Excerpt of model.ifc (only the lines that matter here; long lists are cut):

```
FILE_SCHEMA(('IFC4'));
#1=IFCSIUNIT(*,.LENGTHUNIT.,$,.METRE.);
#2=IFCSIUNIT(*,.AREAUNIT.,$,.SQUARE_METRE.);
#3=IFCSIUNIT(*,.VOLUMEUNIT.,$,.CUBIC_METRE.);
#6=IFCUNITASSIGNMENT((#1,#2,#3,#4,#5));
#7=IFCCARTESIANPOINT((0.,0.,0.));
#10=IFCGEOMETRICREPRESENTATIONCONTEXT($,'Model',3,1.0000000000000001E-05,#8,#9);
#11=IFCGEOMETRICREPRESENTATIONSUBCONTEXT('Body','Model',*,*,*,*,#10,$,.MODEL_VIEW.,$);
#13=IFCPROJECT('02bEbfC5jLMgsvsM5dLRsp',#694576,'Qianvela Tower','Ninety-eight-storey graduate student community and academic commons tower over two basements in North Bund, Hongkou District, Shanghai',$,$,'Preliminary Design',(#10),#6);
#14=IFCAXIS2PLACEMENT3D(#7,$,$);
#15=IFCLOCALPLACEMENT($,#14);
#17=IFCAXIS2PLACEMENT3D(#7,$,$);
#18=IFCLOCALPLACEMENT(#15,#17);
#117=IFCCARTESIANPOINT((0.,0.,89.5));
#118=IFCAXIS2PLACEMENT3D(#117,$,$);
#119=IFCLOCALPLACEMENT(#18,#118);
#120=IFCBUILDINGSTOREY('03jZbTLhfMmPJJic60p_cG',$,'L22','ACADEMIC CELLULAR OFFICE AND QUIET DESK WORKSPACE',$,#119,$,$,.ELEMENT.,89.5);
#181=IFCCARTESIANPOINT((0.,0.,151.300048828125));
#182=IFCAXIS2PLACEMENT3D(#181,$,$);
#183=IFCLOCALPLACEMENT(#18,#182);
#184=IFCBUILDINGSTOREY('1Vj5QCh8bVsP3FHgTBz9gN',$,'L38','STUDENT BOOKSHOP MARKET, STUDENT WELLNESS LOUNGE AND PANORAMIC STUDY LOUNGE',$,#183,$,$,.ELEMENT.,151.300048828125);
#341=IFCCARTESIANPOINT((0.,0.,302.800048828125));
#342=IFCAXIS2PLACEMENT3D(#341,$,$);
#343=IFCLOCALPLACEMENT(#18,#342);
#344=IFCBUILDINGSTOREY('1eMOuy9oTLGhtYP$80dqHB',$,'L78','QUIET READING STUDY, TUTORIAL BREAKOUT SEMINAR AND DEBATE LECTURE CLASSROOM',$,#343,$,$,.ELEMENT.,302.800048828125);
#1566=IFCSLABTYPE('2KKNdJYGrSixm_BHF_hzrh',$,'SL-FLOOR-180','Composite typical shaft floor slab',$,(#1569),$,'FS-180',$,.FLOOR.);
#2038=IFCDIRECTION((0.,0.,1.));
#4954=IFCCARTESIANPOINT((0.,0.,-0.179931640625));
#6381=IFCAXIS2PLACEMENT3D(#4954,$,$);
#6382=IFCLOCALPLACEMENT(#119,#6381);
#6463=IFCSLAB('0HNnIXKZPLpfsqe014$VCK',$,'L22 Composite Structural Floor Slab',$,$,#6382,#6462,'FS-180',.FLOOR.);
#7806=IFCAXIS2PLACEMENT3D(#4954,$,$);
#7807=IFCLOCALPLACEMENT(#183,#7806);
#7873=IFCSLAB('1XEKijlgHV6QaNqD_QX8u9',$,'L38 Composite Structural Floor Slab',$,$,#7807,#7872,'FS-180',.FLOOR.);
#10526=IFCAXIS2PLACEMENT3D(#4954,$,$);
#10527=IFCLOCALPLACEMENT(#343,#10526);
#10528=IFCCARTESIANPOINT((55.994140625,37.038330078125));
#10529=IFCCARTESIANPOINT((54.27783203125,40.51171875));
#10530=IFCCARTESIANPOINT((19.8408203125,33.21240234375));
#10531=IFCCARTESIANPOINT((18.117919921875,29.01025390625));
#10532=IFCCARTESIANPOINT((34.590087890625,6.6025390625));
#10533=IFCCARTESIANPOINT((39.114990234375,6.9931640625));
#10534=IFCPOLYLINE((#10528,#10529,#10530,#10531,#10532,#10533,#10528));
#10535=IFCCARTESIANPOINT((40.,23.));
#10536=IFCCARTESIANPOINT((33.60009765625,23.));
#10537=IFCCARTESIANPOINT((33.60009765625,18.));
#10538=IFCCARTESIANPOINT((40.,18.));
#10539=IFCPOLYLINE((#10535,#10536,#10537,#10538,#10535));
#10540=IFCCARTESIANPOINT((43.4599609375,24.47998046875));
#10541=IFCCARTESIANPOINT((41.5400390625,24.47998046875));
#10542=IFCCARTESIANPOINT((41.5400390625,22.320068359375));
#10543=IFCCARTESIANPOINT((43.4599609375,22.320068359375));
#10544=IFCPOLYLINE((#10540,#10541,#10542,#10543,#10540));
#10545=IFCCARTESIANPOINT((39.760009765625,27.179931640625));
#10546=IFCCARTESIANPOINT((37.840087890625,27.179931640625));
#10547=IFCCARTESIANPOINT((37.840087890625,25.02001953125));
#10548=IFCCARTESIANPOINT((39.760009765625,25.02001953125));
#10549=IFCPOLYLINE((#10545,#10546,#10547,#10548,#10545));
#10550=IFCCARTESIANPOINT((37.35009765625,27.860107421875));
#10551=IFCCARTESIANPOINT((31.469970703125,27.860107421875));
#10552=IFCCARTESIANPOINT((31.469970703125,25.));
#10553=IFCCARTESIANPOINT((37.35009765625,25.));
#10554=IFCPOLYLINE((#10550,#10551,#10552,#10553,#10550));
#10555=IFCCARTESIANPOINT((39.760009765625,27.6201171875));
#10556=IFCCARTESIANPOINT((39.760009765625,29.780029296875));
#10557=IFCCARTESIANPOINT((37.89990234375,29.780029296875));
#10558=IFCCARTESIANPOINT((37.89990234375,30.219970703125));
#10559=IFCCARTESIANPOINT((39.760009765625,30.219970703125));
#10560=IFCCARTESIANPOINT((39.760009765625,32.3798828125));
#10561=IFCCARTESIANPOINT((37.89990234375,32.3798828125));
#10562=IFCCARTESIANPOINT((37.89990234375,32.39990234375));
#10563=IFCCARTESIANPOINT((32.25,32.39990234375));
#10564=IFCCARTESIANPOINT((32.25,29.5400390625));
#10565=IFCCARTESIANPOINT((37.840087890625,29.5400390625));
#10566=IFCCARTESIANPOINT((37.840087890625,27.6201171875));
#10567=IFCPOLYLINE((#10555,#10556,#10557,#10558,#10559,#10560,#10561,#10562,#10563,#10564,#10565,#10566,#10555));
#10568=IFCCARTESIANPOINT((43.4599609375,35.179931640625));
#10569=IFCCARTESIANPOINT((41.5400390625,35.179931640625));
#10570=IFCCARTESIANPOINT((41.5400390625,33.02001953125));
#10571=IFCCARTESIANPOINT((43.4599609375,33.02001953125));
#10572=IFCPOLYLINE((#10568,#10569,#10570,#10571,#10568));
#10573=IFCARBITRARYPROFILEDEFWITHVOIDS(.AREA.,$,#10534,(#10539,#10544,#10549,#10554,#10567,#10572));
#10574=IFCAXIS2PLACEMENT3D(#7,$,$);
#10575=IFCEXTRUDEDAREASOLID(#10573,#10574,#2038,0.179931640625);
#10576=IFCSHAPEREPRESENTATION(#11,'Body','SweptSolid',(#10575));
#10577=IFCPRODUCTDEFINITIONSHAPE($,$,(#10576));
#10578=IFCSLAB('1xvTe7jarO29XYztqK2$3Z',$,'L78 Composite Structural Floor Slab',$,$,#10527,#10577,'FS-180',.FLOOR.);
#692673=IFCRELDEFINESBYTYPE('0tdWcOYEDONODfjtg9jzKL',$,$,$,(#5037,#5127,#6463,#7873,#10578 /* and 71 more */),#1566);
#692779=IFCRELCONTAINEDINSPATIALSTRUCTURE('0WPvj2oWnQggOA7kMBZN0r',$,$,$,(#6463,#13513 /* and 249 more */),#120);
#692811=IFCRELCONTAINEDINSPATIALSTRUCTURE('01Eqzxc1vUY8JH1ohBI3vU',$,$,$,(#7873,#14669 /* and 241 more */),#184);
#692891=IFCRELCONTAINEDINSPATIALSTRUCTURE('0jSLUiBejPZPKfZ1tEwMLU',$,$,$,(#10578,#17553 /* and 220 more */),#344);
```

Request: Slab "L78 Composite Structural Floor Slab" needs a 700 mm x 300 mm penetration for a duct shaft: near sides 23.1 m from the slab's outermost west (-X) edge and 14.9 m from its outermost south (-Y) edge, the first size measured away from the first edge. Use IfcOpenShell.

```python
import numpy as np
import ifcopenshell
import ifcopenshell.api.feature
import ifcopenshell.api.geometry
import ifcopenshell.api.root
import ifcopenshell.geom
import ifcopenshell.util.placement
import ifcopenshell.util.representation
import ifcopenshell.util.shape
import ifcopenshell.util.unit

model = ifcopenshell.open("model.ifc")
unit_scale = ifcopenshell.util.unit.calculate_unit_scale(model)
settings = ifcopenshell.geom.settings()


def volume(element):
    """Net volume in cubic metres, openings subtracted."""
    shape = ifcopenshell.geom.create_shape(settings, element)
    return ifcopenshell.util.shape.get_volume(shape.geometry)


slab = model.by_guid("1xvTe7jarO29XYztqK2$3Z")
before = volume(slab)

# Extent in the slab's own axes, in metres. The edges named are its -X and -Y sides.
slab_shape = ifcopenshell.geom.create_shape(settings, slab)
vertices = ifcopenshell.util.shape.get_vertices(slab_shape.geometry)
x_min, y_min, bottom = vertices.min(axis=0)
top = vertices[:, 2].max()

opening = ifcopenshell.api.root.create_entity(model, ifc_class="IfcOpeningElement", name="Duct shaft opening", predefined_type="OPENING")
context = ifcopenshell.util.representation.get_context(model, "Model", "Body", "MODEL_VIEW")
width, depth = 0.7, 0.3
outline = [(0.0, 0.0), (width, 0.0), (width, depth), (0.0, depth), (0.0, 0.0)]
# Overshoot both faces by 50 mm so the cut is clean.
shape = ifcopenshell.api.geometry.add_slab_representation(
    model, context=context, depth=top - bottom + 0.1, polyline=outline
)
ifcopenshell.api.geometry.assign_representation(model, product=opening, representation=shape)

matrix = ifcopenshell.util.placement.get_local_placement(slab.ObjectPlacement)
matrix[:, 3] = matrix @ np.append(np.array([x_min + 23.1, y_min + 14.9, bottom - 0.05]) / unit_scale, 1.0)
ifcopenshell.api.geometry.edit_object_placement(model, product=opening, matrix=matrix, is_si=False)
ifcopenshell.api.feature.add_feature(model, feature=opening, element=slab)

after = volume(slab)

print(f"slab volume {before:.3f} -> {after:.3f} m3")

model.write("model_edited.ifc")
```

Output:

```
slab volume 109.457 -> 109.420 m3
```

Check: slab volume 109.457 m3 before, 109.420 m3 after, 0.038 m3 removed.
